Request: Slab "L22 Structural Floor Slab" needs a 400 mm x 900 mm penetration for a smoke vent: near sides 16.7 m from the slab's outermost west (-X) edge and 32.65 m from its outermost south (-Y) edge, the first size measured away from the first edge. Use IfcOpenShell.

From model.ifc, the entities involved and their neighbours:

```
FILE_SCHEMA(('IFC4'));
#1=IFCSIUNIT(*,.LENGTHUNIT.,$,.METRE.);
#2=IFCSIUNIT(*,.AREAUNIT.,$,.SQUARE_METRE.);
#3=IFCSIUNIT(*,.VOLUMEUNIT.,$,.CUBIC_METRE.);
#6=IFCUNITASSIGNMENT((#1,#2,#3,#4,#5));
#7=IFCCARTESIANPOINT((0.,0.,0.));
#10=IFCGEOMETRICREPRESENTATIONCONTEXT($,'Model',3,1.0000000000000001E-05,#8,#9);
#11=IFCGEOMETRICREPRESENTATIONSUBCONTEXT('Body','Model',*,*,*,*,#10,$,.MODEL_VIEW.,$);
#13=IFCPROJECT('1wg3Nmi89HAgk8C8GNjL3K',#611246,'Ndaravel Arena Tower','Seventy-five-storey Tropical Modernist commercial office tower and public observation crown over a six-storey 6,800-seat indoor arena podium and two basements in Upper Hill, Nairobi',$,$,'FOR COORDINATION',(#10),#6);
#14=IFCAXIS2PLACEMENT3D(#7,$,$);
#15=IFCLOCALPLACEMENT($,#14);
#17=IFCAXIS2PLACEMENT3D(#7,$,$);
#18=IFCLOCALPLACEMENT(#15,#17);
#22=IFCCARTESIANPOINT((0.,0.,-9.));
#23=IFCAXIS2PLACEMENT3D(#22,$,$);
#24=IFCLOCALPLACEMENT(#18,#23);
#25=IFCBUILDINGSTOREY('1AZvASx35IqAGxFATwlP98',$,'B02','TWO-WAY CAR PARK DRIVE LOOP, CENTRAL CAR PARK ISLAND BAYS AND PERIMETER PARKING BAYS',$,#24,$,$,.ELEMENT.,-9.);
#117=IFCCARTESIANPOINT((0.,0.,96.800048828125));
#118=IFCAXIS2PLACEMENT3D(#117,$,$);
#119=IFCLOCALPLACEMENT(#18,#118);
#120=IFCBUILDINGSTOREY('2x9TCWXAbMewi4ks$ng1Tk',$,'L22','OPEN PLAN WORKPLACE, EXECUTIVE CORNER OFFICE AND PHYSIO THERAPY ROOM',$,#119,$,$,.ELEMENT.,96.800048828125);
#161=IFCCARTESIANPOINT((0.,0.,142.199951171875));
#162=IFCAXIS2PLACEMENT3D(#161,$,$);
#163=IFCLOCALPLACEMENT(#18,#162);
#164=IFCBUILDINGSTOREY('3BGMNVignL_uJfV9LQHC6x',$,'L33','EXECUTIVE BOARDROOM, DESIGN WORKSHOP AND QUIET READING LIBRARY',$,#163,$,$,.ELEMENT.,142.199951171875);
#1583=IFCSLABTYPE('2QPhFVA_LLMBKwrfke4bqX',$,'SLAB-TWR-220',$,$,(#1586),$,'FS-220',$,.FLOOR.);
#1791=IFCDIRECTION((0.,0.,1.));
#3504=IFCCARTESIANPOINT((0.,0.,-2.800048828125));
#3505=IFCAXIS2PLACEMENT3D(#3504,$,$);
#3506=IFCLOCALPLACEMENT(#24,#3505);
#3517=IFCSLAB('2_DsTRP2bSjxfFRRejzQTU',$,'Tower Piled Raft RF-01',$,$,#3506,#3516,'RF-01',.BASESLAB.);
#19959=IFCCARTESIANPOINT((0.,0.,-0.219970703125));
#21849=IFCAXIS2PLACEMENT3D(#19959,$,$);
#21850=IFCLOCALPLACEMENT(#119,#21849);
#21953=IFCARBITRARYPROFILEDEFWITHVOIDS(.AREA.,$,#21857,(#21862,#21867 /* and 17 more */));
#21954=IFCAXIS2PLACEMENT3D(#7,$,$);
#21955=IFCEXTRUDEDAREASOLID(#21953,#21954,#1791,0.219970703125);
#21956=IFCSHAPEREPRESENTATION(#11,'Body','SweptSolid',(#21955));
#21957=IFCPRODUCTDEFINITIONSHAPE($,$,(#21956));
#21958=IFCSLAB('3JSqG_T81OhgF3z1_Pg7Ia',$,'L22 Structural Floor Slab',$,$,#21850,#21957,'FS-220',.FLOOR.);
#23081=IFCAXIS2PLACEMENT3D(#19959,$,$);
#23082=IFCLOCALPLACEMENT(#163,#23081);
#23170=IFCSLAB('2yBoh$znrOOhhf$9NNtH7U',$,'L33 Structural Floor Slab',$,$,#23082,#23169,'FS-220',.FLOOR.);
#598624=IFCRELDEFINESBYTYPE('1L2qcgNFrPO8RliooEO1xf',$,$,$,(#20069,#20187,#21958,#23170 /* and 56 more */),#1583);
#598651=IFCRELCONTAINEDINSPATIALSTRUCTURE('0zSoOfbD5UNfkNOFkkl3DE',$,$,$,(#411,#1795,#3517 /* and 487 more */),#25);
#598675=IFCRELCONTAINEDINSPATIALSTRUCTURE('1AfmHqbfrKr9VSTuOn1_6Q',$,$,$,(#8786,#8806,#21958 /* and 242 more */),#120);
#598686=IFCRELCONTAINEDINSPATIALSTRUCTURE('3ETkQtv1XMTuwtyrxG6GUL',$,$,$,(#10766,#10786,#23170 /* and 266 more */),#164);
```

```python
import numpy as np
import ifcopenshell
import ifcopenshell.api.feature
import ifcopenshell.api.geometry
import ifcopenshell.api.root
import ifcopenshell.geom
import ifcopenshell.util.placement
import ifcopenshell.util.representation
import ifcopenshell.util.shape
import ifcopenshell.util.unit

model = ifcopenshell.open("model.ifc")
unit_scale = ifcopenshell.util.unit.calculate_unit_scale(model)
settings = ifcopenshell.geom.settings()


def volume(element):
    """Net volume in cubic metres, openings subtracted."""
    shape = ifcopenshell.geom.create_shape(settings, element)
    return ifcopenshell.util.shape.get_volume(shape.geometry)


slab = model.by_guid("3JSqG_T81OhgF3z1_Pg7Ia")
before = volume(slab)

# Extent in the slab's own axes, in metres. The edges named are its -X and -Y sides.
slab_shape = ifcopenshell.geom.create_shape(settings, slab)
vertices = ifcopenshell.util.shape.get_vertices(slab_shape.geometry)
x_min, y_min, bottom = vertices.min(axis=0)
top = vertices[:, 2].max()

opening = ifcopenshell.api.root.create_entity(model, ifc_class="IfcOpeningElement", name="Smoke vent opening", predefined_type="OPENING")
context = ifcopenshell.util.representation.get_context(model, "Model", "Body", "MODEL_VIEW")
width, depth = 0.4, 0.9
outline = [(0.0, 0.0), (width, 0.0), (width, depth), (0.0, depth), (0.0, 0.0)]
# Overshoot both faces by 50 mm so the cut is clean.
shape = ifcopenshell.api.geometry.add_slab_representation(
    model, context=context, depth=top - bottom + 0.1, polyline=outline
)
ifcopenshell.api.geometry.assign_representation(model, product=opening, representation=shape)

matrix = ifcopenshell.util.placement.get_local_placement(slab.ObjectPlacement)
matrix[:, 3] = matrix @ np.append(np.array([x_min + 16.7, y_min + 32.65, bottom - 0.05]) / unit_scale, 1.0)
ifcopenshell.api.geometry.edit_object_placement(model, product=opening, matrix=matrix, is_si=False)
ifcopenshell.api.feature.add_feature(model, feature=opening, element=slab)

after = volume(slab)

print(f"slab volume {before:.3f} -> {after:.3f} m3")

model.write("model_v2.ifc")
```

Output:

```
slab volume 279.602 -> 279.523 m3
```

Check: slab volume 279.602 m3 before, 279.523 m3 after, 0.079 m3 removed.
